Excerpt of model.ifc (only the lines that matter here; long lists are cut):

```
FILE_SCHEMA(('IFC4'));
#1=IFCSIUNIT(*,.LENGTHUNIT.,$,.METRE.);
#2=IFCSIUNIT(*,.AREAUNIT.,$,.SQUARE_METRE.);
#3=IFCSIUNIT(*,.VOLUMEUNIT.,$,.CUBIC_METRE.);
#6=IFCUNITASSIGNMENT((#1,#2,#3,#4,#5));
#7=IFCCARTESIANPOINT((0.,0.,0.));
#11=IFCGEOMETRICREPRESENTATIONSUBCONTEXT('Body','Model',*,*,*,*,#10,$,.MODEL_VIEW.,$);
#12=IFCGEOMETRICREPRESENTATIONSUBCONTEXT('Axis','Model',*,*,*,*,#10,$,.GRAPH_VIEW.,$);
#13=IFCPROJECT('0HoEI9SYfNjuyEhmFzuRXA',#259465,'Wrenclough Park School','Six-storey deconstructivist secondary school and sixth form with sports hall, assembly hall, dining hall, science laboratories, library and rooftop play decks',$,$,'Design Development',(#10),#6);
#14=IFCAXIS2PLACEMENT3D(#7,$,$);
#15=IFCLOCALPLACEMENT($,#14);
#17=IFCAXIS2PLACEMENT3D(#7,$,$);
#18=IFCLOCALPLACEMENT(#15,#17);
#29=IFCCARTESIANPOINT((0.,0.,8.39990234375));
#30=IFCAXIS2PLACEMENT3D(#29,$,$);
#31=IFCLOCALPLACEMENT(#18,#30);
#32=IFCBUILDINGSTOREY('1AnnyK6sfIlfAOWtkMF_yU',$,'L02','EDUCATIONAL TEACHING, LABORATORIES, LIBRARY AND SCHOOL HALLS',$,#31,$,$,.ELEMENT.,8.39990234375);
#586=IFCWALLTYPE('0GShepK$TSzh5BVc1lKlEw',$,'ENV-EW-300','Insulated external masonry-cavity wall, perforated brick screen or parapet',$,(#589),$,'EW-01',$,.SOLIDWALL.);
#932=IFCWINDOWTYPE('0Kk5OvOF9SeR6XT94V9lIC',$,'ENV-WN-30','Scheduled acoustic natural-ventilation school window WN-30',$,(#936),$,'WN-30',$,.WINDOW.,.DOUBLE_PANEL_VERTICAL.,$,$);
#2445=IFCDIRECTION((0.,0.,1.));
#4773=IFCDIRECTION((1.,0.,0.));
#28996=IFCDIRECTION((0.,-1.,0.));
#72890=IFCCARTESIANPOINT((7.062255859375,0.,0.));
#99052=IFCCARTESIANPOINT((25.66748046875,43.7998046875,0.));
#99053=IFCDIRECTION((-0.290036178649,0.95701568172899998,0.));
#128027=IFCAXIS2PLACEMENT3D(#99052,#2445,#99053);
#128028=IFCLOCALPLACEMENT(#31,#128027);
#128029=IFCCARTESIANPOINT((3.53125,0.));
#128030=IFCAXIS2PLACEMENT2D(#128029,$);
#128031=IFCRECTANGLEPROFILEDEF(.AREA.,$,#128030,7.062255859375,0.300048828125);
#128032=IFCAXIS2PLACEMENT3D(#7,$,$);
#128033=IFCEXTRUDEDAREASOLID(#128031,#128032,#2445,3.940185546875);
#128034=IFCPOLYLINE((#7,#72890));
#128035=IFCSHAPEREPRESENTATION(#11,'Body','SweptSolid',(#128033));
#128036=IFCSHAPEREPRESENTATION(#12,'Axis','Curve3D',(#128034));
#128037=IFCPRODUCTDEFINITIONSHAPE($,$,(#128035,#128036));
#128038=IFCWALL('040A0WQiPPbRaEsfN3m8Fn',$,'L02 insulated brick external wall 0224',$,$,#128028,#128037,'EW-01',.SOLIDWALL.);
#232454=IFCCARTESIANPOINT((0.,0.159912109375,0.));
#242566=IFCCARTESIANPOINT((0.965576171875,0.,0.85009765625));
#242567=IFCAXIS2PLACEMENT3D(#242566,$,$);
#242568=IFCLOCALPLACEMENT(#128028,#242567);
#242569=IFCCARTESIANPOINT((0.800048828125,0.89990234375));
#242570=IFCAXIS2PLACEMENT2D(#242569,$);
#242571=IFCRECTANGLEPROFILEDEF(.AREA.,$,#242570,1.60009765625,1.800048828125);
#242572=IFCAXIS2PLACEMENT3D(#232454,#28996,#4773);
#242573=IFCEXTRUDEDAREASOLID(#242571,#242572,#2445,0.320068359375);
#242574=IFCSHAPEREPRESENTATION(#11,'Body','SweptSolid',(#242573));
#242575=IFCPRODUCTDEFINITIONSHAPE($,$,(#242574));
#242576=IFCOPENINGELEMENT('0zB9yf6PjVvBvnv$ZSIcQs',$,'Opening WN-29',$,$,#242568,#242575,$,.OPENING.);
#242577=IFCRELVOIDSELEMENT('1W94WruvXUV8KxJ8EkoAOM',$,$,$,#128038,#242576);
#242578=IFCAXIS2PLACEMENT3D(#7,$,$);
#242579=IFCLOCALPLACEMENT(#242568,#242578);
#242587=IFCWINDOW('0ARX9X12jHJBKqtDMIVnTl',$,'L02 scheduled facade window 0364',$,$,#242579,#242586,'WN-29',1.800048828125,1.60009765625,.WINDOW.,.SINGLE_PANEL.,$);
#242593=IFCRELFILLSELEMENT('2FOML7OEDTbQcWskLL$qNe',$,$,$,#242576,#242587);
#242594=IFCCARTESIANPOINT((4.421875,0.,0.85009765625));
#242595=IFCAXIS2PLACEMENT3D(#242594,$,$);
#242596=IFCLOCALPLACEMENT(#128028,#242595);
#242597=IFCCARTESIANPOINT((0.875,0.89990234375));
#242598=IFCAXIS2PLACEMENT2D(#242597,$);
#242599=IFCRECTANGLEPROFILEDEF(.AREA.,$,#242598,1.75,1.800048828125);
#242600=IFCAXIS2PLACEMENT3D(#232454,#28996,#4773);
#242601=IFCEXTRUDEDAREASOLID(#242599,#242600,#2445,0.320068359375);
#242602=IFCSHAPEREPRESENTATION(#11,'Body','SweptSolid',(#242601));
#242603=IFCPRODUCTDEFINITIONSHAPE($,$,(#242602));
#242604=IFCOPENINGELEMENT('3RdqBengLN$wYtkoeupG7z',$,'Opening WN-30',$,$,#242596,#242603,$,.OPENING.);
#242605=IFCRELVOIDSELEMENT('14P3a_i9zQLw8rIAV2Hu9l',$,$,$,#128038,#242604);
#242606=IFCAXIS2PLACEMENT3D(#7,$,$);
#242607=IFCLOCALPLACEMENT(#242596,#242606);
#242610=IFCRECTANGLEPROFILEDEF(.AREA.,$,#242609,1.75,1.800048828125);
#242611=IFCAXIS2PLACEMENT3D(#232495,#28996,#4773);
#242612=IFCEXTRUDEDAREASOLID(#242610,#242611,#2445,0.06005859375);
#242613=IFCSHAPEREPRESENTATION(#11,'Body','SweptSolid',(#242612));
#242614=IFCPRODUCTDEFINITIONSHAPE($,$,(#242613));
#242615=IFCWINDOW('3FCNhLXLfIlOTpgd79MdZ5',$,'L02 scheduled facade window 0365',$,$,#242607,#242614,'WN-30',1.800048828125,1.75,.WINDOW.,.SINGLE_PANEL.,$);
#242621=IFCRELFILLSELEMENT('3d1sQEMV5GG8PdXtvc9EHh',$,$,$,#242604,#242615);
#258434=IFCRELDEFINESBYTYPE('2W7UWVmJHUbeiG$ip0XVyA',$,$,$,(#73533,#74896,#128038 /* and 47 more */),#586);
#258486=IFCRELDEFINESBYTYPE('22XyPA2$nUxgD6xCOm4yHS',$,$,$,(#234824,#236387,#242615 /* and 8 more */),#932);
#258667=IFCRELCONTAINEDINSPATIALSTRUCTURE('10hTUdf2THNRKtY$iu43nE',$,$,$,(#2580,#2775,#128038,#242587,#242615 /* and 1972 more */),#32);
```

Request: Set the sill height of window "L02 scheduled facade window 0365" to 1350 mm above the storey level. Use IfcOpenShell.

```python
import numpy as np
import ifcopenshell
import ifcopenshell.api.geometry
import ifcopenshell.geom
import ifcopenshell.util.element
import ifcopenshell.util.placement
import ifcopenshell.util.shape
import ifcopenshell.util.unit

model = ifcopenshell.open("model.ifc")
unit_scale = ifcopenshell.util.unit.calculate_unit_scale(model)

window = model.by_guid("3FCNhLXLfIlOTpgd79MdZ5")
opening = window.FillsVoids[0].RelatingOpeningElement
storey = ifcopenshell.util.element.get_container(window, ifc_class="IfcBuildingStorey")
level = ifcopenshell.util.placement.get_local_placement(storey.ObjectPlacement)[2, 3]

# The opening's origin need not be at the sill, so measure its lowest point.
shape = ifcopenshell.geom.create_shape(ifcopenshell.geom.settings(), opening)
bottom = ifcopenshell.util.shape.get_shape_bottom_elevation(shape, shape.geometry) / unit_scale
dz = level + 1.35 - bottom

shift = np.array([0.0, 0.0, dz])
# The window is placed relative to its opening, so it follows when the opening moves.
matrix = ifcopenshell.util.placement.get_local_placement(opening.ObjectPlacement)
matrix[:3, 3] += shift
ifcopenshell.api.geometry.edit_object_placement(
    model, product=opening, matrix=matrix, is_si=False, should_transform_children=True
)

print(f"moved by {dz * unit_scale:+.3f} m")

model.write("model_rev.ifc")
```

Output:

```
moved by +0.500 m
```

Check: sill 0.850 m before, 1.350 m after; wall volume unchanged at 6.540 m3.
